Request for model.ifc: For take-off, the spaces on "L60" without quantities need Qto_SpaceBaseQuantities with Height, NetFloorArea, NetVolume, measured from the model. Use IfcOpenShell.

First a look at what the model holds.

```python
import ifcopenshell
import ifcopenshell.util.element
import ifcopenshell.util.unit

model = ifcopenshell.open("model.ifc")
print(model.schema)
for unit_type in ("LENGTHUNIT", "AREAUNIT", "VOLUMEUNIT"):
    print(unit_type, ifcopenshell.util.unit.calculate_unit_scale(model, unit_type))
storey = next(s for s in model.by_type("IfcBuildingStorey") if s.Name == "L60")
spaces = [e for e in ifcopenshell.util.element.get_decomposition(storey) if e.is_a("IfcSpace")]
for e in sorted(spaces, key=lambda e: e.id()):
    print(e.id(), e.is_a(), e.Name, list(ifcopenshell.util.element.get_psets(e, qtos_only=True)), sep=" | ")
```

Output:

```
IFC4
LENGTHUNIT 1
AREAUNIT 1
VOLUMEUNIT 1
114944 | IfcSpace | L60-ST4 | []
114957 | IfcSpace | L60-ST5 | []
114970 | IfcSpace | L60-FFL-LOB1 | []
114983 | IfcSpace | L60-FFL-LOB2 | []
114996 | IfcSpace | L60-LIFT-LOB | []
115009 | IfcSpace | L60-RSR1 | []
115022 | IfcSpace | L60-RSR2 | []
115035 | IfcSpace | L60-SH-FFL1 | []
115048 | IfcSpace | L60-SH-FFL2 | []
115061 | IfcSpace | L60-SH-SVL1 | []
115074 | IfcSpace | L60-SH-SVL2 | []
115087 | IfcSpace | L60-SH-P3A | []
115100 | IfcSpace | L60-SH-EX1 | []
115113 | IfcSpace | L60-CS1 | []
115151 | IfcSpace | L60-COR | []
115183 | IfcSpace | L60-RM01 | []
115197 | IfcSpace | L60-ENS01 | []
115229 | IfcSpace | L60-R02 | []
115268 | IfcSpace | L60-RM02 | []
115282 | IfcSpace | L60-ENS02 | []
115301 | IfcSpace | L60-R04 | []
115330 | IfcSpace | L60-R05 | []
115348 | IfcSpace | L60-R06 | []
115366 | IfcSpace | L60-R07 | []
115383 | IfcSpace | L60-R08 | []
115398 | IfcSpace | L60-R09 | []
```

```python
import ifcopenshell
import ifcopenshell.api.pset
import ifcopenshell.geom
import ifcopenshell.util.element
import ifcopenshell.util.shape
import ifcopenshell.util.unit

model = ifcopenshell.open("model.ifc")
unit_scale = ifcopenshell.util.unit.calculate_unit_scale(model)
area_scale = ifcopenshell.util.unit.calculate_unit_scale(model, "AREAUNIT")
volume_scale = ifcopenshell.util.unit.calculate_unit_scale(model, "VOLUMEUNIT")
settings = ifcopenshell.geom.settings()

storey = next(s for s in model.by_type("IfcBuildingStorey") if s.Name == "L60")
spaces = [e for e in ifcopenshell.util.element.get_decomposition(storey) if e.is_a("IfcSpace")]

for e in sorted(spaces, key=lambda e: e.id()):
    if ifcopenshell.util.element.get_psets(e, qtos_only=True, should_inherit=False):
        continue
    # Geometry comes back in metres, in the element's own axes.
    shape = ifcopenshell.geom.create_shape(settings, e)
    values = {
        "Height": ifcopenshell.util.shape.get_z(shape.geometry) / unit_scale,
        "NetFloorArea": ifcopenshell.util.shape.get_footprint_area(shape.geometry) / area_scale,
        "NetVolume": ifcopenshell.util.shape.get_volume(shape.geometry) / volume_scale,
    }
    qto = ifcopenshell.api.pset.add_qto(model, product=e, name="Qto_SpaceBaseQuantities")
    ifcopenshell.api.pset.edit_qto(model, qto=qto, properties=values)
    print(e.id(), {k: round(v, 3) for k, v in values.items()})

model.write("model_v2.ifc")
```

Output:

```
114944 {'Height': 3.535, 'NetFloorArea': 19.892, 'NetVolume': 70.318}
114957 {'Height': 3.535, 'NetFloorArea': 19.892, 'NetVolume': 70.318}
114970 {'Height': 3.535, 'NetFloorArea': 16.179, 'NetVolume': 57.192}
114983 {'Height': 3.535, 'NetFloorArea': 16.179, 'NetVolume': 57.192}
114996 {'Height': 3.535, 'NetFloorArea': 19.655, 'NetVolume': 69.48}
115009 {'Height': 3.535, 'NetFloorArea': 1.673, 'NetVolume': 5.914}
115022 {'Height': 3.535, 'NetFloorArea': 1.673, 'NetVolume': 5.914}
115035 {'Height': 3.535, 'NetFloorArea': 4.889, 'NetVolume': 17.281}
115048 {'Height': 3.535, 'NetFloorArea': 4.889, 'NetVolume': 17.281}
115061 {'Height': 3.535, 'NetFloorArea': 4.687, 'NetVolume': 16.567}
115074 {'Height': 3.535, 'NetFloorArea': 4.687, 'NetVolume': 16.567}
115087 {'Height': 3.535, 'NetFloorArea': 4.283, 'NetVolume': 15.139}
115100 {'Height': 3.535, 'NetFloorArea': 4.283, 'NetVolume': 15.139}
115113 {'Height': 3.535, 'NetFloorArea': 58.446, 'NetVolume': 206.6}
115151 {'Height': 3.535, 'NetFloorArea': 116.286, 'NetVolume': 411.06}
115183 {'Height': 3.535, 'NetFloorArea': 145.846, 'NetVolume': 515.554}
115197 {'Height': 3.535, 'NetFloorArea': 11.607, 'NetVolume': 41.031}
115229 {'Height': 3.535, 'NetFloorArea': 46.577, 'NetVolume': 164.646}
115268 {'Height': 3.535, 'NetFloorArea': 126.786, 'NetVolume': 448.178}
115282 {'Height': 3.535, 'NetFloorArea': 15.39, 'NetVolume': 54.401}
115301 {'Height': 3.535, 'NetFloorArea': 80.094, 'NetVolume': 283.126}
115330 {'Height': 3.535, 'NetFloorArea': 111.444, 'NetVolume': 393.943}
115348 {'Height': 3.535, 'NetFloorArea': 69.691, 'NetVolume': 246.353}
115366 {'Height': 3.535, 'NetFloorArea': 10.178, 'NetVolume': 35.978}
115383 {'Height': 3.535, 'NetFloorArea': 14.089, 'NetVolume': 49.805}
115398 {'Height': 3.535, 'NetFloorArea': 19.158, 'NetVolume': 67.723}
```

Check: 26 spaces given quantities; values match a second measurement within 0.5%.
